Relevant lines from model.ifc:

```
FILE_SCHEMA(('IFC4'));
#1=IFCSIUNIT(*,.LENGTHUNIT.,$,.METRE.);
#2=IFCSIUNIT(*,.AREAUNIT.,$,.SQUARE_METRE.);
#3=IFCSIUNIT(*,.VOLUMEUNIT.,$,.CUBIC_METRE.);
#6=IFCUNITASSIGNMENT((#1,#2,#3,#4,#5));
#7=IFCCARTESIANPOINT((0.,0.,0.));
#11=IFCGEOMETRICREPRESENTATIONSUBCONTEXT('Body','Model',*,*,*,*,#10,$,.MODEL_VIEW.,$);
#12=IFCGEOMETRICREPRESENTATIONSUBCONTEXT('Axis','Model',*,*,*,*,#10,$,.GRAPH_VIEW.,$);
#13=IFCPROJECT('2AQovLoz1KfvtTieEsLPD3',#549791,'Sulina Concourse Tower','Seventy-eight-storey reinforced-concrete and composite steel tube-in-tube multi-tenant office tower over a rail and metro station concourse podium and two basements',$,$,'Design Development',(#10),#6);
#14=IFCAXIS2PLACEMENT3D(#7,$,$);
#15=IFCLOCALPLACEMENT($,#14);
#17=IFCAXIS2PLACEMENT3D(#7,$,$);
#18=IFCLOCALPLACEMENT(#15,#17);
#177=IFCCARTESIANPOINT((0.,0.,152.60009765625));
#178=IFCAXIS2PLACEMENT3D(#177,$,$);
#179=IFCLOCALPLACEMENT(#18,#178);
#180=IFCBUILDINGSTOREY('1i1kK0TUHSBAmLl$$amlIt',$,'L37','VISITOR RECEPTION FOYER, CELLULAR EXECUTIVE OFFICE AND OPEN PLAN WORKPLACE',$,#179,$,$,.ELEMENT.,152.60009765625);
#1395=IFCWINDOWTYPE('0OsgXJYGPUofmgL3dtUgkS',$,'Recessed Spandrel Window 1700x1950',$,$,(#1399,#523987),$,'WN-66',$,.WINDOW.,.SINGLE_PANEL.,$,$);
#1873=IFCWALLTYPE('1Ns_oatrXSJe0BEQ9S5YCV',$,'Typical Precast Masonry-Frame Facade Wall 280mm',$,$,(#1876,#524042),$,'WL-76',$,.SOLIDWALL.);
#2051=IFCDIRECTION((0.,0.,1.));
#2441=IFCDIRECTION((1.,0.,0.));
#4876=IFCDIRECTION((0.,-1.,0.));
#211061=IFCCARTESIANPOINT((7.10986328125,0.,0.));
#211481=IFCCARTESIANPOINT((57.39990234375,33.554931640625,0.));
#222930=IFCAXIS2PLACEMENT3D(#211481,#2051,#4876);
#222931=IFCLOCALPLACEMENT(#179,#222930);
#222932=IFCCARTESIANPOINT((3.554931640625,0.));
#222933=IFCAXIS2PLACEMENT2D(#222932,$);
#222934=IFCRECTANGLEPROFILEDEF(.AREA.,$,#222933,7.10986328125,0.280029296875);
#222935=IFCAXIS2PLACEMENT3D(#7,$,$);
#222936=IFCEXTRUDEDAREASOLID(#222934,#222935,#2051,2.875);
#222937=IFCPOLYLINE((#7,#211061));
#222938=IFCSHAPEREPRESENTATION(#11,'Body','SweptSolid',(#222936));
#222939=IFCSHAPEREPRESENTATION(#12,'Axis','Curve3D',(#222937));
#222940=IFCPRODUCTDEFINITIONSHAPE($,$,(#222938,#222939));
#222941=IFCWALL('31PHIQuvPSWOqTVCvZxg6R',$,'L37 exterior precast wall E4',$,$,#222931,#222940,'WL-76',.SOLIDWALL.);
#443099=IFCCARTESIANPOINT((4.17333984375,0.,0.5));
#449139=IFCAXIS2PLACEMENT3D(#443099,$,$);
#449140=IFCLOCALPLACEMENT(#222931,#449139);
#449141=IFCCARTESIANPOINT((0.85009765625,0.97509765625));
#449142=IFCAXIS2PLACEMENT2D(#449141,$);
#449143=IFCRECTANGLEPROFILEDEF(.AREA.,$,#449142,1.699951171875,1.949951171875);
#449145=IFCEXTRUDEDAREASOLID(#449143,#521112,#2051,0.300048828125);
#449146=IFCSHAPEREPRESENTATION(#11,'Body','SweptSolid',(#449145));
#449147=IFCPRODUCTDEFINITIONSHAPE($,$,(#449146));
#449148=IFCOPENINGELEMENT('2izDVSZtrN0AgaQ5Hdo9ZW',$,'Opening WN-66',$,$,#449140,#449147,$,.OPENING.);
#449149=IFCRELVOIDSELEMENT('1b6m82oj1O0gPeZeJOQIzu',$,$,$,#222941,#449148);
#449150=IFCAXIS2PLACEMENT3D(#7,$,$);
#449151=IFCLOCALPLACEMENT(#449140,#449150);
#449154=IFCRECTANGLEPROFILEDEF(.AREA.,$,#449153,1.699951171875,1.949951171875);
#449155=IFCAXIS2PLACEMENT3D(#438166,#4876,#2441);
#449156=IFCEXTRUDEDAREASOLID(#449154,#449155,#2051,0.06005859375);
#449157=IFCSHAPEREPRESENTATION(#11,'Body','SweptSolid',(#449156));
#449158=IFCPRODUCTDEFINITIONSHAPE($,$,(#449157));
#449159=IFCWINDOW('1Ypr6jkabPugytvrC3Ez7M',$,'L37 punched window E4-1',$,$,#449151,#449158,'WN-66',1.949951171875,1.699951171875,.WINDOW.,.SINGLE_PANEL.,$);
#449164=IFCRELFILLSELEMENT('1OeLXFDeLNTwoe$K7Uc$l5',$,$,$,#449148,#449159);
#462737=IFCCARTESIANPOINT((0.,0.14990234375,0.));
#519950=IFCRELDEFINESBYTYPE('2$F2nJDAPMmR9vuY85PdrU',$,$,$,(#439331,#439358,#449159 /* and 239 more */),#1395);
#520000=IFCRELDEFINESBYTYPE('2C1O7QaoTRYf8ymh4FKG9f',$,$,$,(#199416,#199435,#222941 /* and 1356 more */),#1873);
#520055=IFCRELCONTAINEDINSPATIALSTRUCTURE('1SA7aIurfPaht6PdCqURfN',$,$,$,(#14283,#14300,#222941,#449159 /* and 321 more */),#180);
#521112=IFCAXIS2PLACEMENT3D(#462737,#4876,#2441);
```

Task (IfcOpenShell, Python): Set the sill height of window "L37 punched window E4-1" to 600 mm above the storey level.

```python
import numpy as np
import ifcopenshell
import ifcopenshell.api.geometry
import ifcopenshell.geom
import ifcopenshell.util.element
import ifcopenshell.util.placement
import ifcopenshell.util.shape
import ifcopenshell.util.unit

model = ifcopenshell.open("model.ifc")
unit_scale = ifcopenshell.util.unit.calculate_unit_scale(model)

window = model.by_guid("1Ypr6jkabPugytvrC3Ez7M")
opening = window.FillsVoids[0].RelatingOpeningElement
storey = ifcopenshell.util.element.get_container(window, ifc_class="IfcBuildingStorey")
level = ifcopenshell.util.placement.get_local_placement(storey.ObjectPlacement)[2, 3]

# The opening's origin need not be at the sill, so measure its lowest point.
shape = ifcopenshell.geom.create_shape(ifcopenshell.geom.settings(), opening)
bottom = ifcopenshell.util.shape.get_shape_bottom_elevation(shape, shape.geometry) / unit_scale
dz = level + 0.6 - bottom

shift = np.array([0.0, 0.0, dz])
# The window is placed relative to its opening, so it follows when the opening moves.
matrix = ifcopenshell.util.placement.get_local_placement(opening.ObjectPlacement)
matrix[:3, 3] += shift
ifcopenshell.api.geometry.edit_object_placement(
    model, product=opening, matrix=matrix, is_si=False, should_transform_children=True
)

print(f"moved by {dz * unit_scale:+.3f} m")

model.write("model_rev.ifc")
```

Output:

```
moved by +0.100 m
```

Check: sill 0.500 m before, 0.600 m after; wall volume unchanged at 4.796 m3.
